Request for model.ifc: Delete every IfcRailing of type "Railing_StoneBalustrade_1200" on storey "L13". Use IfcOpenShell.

First a look at what the model holds.

```python
import ifcopenshell
import ifcopenshell.util.element

model = ifcopenshell.open("model.ifc")
print(model.schema)
storey = next(s for s in model.by_type("IfcBuildingStorey") if s.Name == "L13")
railings = [e for e in ifcopenshell.util.element.get_decomposition(storey) if e.is_a("IfcRailing")]
seen = {}
for e in railings:
    element_type = ifcopenshell.util.element.get_type(e)
    name = element_type.Name if element_type not in (None, e) else None
    seen[name] = seen.get(name, 0) + 1
for name, count in sorted(seen.items(), key=str):
    print(count, "x", name)
```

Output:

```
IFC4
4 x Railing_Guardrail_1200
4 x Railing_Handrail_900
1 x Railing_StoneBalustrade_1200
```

```python
import ifcopenshell
import ifcopenshell.api.root
import ifcopenshell.util.element

model = ifcopenshell.open("model.ifc")

storey = next(s for s in model.by_type("IfcBuildingStorey") if s.Name == "L13")
railings = [e for e in ifcopenshell.util.element.get_decomposition(storey) if e.is_a("IfcRailing")]
targets = [e for e in railings if (t := ifcopenshell.util.element.get_type(e)) not in (None, e) and t.Name == "Railing_StoneBalustrade_1200"]

for e in targets:
    ifcopenshell.api.root.remove_product(model, product=e)
print(len(targets), "removed")

model.write("model_v2.ifc")
```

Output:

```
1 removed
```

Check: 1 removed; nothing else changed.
